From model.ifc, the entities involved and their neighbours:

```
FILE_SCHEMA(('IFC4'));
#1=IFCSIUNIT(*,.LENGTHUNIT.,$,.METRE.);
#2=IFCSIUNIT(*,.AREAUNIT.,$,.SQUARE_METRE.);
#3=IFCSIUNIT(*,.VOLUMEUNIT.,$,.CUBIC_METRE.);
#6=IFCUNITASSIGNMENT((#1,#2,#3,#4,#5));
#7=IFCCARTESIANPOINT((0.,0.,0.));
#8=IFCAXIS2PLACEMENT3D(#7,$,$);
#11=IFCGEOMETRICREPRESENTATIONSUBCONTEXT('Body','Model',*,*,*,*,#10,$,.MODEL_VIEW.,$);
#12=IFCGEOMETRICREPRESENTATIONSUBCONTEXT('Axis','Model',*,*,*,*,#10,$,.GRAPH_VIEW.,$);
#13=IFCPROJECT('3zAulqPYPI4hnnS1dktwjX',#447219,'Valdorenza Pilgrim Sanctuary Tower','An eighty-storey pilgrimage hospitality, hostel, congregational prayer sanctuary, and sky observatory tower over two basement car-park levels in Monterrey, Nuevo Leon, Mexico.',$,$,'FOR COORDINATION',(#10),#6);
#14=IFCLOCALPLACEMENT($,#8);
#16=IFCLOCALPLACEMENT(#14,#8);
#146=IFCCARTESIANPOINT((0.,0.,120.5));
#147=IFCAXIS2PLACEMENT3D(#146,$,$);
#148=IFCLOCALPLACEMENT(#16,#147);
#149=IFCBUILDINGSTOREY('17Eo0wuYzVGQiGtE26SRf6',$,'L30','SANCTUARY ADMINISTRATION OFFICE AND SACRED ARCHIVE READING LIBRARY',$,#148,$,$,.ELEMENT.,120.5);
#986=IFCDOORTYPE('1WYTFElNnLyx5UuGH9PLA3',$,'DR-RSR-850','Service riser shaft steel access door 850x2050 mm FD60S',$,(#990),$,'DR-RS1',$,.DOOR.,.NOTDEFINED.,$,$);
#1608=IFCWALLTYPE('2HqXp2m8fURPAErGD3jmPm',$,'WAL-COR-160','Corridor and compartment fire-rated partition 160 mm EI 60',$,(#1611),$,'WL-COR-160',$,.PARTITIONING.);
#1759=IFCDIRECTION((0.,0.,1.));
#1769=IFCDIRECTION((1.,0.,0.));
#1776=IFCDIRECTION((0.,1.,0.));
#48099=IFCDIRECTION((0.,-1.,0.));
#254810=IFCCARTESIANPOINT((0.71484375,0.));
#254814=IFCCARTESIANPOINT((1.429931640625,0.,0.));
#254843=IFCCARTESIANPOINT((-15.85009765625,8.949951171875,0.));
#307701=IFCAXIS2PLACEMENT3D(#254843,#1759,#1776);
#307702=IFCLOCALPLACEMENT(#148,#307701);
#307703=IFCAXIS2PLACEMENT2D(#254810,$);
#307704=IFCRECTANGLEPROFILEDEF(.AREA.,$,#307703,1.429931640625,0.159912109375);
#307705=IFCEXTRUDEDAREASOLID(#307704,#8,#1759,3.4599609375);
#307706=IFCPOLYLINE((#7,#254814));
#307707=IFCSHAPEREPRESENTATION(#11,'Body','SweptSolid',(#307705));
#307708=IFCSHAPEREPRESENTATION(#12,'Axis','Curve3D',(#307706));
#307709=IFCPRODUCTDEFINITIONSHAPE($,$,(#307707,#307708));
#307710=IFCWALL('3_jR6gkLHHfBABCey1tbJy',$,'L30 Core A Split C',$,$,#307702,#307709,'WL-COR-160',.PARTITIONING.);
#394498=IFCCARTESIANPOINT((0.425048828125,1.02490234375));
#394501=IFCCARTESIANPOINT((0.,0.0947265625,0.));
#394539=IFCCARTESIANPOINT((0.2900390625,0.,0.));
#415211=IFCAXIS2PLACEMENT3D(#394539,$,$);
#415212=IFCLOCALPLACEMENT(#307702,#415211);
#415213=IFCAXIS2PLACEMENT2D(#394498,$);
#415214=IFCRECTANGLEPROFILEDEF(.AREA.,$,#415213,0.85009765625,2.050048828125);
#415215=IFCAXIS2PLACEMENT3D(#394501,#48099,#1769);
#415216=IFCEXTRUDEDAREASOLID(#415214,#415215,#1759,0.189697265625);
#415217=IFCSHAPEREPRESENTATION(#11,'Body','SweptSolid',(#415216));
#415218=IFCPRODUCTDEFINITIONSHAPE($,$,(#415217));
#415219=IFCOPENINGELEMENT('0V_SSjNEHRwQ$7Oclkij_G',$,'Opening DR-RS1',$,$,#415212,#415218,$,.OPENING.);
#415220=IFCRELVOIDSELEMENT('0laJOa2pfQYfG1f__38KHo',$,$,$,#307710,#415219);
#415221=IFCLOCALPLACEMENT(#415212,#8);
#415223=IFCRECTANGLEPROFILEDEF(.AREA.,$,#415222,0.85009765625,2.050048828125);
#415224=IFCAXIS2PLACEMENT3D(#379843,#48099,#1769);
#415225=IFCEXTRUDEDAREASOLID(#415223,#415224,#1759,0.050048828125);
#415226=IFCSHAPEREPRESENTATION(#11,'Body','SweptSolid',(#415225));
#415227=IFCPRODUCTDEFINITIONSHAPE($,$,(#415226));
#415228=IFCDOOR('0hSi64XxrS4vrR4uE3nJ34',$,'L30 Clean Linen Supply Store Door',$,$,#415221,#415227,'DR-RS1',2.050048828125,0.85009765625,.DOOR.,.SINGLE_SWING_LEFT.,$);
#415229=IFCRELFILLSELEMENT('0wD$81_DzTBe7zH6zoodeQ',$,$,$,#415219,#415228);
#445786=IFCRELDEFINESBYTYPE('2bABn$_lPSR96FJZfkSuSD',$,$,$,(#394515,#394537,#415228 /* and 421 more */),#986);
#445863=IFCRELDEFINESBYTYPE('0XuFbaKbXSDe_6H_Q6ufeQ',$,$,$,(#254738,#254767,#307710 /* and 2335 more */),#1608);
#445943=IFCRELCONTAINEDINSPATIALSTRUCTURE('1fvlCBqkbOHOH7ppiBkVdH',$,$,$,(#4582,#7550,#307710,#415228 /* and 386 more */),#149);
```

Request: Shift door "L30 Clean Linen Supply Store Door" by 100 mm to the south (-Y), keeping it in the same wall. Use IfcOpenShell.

```python
import ifcopenshell
import ifcopenshell.api.geometry
import ifcopenshell.util.placement

model = ifcopenshell.open("model.ifc")

door = model.by_id(415228)
opening = door.FillsVoids[0].RelatingOpeningElement
wall = opening.VoidsElements[0].RelatingBuildingElement

wall_matrix = ifcopenshell.util.placement.get_local_placement(wall.ObjectPlacement)
shift = wall_matrix[:3, 0] * -0.1
before = ifcopenshell.util.placement.get_local_placement(door.ObjectPlacement)[:3, 3].copy()

# The door is placed relative to its opening, so it follows when the opening moves.
matrix = ifcopenshell.util.placement.get_local_placement(opening.ObjectPlacement)
matrix[:3, 3] += shift
ifcopenshell.api.geometry.edit_object_placement(
    model, product=opening, matrix=matrix, is_si=False, should_transform_children=True
)

after = ifcopenshell.util.placement.get_local_placement(door.ObjectPlacement)[:3, 3]
print("door moved by", (after - before).round(3) + 0.0)

model.write("model_v2.ifc")
```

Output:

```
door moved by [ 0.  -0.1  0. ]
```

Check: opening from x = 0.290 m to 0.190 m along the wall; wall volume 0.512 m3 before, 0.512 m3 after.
